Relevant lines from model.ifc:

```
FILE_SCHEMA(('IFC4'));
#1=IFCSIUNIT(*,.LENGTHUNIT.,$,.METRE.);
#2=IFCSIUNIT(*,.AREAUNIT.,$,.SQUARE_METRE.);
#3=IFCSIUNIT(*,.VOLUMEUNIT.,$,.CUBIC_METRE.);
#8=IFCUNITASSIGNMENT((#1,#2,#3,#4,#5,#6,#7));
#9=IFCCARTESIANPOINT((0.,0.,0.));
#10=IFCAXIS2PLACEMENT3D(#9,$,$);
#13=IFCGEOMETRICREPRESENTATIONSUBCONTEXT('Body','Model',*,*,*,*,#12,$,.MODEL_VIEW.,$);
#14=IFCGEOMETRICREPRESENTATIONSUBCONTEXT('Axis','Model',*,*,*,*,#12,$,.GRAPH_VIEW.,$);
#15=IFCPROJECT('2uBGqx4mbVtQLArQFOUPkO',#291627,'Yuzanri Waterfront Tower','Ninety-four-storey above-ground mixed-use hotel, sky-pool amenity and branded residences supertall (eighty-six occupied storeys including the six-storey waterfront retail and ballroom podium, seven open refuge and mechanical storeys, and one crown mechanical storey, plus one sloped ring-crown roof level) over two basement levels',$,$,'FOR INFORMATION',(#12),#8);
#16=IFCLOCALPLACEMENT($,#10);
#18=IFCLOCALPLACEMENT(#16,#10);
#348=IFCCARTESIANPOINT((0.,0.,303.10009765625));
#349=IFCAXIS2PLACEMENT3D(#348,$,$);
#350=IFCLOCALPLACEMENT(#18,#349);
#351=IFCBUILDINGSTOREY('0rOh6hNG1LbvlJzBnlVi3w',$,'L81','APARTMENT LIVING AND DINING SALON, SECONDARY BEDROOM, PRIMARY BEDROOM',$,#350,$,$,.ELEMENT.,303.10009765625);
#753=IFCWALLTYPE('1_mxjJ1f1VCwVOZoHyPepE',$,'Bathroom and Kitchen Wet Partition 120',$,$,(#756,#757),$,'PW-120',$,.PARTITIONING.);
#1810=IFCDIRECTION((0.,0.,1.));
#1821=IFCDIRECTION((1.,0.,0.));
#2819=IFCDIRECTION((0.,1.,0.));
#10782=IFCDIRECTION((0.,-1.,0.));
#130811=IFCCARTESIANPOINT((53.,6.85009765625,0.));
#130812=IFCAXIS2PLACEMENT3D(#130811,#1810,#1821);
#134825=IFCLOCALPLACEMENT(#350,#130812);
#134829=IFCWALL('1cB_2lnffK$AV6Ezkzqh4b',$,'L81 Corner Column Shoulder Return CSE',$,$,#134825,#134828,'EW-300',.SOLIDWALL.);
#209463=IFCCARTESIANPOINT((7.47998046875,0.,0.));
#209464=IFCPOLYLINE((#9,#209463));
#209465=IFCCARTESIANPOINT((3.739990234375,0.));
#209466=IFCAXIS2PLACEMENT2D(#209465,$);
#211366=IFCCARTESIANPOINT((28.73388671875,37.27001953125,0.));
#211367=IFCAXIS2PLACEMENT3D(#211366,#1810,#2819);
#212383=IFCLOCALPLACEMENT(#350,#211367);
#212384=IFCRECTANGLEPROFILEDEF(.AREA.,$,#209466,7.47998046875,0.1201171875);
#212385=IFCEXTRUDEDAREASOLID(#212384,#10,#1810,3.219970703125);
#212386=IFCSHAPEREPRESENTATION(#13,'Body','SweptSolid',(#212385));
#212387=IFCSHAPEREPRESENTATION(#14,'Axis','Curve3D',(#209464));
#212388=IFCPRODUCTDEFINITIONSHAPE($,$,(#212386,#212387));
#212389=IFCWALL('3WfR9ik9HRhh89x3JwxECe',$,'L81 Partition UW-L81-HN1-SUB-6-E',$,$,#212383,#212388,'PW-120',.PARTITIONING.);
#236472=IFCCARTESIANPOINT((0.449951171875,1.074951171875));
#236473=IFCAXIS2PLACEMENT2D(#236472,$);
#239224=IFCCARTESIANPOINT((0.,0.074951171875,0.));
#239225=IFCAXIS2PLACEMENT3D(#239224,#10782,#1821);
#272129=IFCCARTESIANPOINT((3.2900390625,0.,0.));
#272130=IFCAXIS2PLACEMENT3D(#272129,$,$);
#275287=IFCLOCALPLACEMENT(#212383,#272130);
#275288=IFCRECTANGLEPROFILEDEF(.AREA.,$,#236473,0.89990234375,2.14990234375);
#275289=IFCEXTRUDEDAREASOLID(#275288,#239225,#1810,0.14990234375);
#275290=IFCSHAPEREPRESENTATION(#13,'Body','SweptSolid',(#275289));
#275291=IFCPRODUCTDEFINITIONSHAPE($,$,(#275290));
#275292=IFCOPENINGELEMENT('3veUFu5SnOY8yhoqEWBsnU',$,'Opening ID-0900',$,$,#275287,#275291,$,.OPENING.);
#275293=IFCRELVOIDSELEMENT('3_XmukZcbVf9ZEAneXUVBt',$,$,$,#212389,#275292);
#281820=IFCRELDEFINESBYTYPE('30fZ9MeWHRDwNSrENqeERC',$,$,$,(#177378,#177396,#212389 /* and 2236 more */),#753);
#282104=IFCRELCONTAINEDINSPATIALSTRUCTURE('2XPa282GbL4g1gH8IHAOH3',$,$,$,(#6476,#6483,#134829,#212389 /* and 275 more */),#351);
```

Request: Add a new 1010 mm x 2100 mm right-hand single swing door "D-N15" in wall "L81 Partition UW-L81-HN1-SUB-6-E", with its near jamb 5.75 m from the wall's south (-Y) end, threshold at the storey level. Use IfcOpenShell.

```python
import numpy as np
import ifcopenshell
import ifcopenshell.api.feature
import ifcopenshell.api.geometry
import ifcopenshell.api.root
import ifcopenshell.api.spatial
import ifcopenshell.geom
import ifcopenshell.util.element
import ifcopenshell.util.placement
import ifcopenshell.util.representation
import ifcopenshell.util.shape
import ifcopenshell.util.unit

model = ifcopenshell.open("model.ifc")
unit_scale = ifcopenshell.util.unit.calculate_unit_scale(model)
settings = ifcopenshell.geom.settings()


def volume(element):
    """Net volume in cubic metres, openings subtracted."""
    shape = ifcopenshell.geom.create_shape(settings, element)
    return ifcopenshell.util.shape.get_volume(shape.geometry)


wall = model.by_guid("3WfR9ik9HRhh89x3JwxECe")
storey = ifcopenshell.util.element.get_container(wall, ifc_class="IfcBuildingStorey")
context = ifcopenshell.util.representation.get_context(model, "Model", "Body", "MODEL_VIEW")
before = volume(wall)

width, height, from_end, sill = 1.01, 2.1, 5.75, 0.0  # metres

# The wall runs along its own X axis, and the end named is its -X end.
wall_shape = ifcopenshell.geom.create_shape(settings, wall)
x, y, z = ifcopenshell.util.shape.get_vertices(wall_shape.geometry).T
start = x.min() + from_end
face, thickness = float(y.min()), float(y.max() - y.min())
wall_matrix = ifcopenshell.util.placement.get_local_placement(wall.ObjectPlacement)
level = ifcopenshell.util.placement.get_local_placement(storey.ObjectPlacement)[2, 3]


def in_wall(x, y):
    """Placement at x, y metres in the wall's axes, at sill height."""
    matrix = wall_matrix.copy()
    matrix[:, 3] = wall_matrix @ np.array([x / unit_scale, y / unit_scale, 0.0, 1.0])
    matrix[2, 3] = level + sill / unit_scale
    return matrix


# Opening: a box that overshoots both wall faces by 50 mm.
opening = ifcopenshell.api.root.create_entity(model, ifc_class="IfcOpeningElement", predefined_type="OPENING")
box = ifcopenshell.api.geometry.add_wall_representation(
    model, context=context, length=width, height=height, thickness=thickness + 0.1
)
ifcopenshell.api.geometry.assign_representation(model, product=opening, representation=box)
ifcopenshell.api.geometry.edit_object_placement(model, product=opening, matrix=in_wall(start, face - 0.05), is_si=False)
ifcopenshell.api.feature.add_feature(model, feature=opening, element=wall)

door = ifcopenshell.api.root.create_entity(model, ifc_class="IfcDoor", name="D-N15", predefined_type="DOOR")
door.OverallWidth, door.OverallHeight = width / unit_scale, height / unit_scale
door.OperationType = "SINGLE_SWING_RIGHT"
body = ifcopenshell.api.geometry.add_door_representation(
    model,
    context=context,
    overall_width=door.OverallWidth,
    overall_height=door.OverallHeight,
    operation_type="SINGLE_SWING_RIGHT",
    lining_properties={"LiningDepth": thickness / unit_scale, "ThresholdDepth": thickness / unit_scale},
)
ifcopenshell.api.geometry.assign_representation(model, product=door, representation=body)
ifcopenshell.api.spatial.assign_container(model, products=[door], relating_structure=storey)
ifcopenshell.api.feature.add_filling(model, opening=opening, element=door)

# The lining spans the wall, so the door starts at the wall face.
ifcopenshell.api.geometry.edit_object_placement(model, product=door, matrix=in_wall(start, face), is_si=False)

after = volume(wall)

print(f"wall volume {before:.3f} -> {after:.3f} m3")

model.write("model_updated.ifc")
```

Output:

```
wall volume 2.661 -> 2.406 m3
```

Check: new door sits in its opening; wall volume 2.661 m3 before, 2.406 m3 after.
